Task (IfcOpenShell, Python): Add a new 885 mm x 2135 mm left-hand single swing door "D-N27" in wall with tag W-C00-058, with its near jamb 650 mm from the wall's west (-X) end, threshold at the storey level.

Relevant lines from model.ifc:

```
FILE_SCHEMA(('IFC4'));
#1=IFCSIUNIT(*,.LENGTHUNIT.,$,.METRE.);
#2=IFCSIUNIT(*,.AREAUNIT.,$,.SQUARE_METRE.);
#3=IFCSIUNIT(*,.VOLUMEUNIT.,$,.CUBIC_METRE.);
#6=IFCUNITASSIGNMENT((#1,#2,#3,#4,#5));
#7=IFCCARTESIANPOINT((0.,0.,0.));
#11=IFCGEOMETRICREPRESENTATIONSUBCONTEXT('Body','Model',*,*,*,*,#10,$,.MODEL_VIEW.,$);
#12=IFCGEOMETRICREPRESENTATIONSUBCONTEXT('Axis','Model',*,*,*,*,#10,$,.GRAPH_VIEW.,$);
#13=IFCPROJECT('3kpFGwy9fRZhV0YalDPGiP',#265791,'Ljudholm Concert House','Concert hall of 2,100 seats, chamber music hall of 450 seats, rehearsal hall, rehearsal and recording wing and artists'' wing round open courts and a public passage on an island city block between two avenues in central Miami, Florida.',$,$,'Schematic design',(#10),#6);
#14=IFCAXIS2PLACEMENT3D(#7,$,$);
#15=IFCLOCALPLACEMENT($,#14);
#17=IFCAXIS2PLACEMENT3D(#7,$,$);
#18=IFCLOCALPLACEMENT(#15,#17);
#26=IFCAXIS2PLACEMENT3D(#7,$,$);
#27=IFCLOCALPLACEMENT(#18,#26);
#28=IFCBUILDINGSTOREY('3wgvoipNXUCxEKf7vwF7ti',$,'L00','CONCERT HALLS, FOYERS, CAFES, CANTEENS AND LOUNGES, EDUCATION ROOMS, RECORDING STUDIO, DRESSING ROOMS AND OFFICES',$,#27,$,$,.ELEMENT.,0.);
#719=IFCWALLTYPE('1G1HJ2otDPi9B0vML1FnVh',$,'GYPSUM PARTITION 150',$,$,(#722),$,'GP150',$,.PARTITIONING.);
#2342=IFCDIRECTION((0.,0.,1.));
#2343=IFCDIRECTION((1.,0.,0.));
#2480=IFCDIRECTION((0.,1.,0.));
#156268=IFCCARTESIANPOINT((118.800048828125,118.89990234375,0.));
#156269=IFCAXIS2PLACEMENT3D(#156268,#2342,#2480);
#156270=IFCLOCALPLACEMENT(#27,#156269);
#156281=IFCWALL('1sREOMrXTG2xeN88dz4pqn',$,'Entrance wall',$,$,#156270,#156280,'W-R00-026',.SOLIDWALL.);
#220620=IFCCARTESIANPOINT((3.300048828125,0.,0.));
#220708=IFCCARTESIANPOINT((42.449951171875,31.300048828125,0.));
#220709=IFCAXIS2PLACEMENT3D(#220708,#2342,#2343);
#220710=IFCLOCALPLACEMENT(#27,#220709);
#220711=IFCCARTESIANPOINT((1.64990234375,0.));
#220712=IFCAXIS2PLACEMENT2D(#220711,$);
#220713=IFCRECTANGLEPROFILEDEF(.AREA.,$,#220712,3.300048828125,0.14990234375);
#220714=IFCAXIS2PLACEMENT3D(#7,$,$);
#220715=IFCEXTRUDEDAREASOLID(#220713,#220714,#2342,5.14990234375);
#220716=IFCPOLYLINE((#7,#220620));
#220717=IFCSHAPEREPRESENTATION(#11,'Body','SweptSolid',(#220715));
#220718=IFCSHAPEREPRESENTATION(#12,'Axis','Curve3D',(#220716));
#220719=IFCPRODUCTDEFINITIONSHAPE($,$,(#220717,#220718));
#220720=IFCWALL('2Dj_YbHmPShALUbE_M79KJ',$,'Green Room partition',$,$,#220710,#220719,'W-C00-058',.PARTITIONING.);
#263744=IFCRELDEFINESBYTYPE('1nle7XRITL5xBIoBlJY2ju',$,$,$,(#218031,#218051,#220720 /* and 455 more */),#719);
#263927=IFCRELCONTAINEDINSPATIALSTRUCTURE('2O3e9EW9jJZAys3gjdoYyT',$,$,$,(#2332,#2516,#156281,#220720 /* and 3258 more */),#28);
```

```python
import numpy as np
import ifcopenshell
import ifcopenshell.api.feature
import ifcopenshell.api.geometry
import ifcopenshell.api.root
import ifcopenshell.api.spatial
import ifcopenshell.geom
import ifcopenshell.util.element
import ifcopenshell.util.placement
import ifcopenshell.util.representation
import ifcopenshell.util.shape
import ifcopenshell.util.unit

model = ifcopenshell.open("model.ifc")
unit_scale = ifcopenshell.util.unit.calculate_unit_scale(model)
settings = ifcopenshell.geom.settings()


def volume(element):
    """Net volume in cubic metres, openings subtracted."""
    shape = ifcopenshell.geom.create_shape(settings, element)
    return ifcopenshell.util.shape.get_volume(shape.geometry)


wall = model.by_id(220720)
storey = ifcopenshell.util.element.get_container(wall, ifc_class="IfcBuildingStorey")
context = ifcopenshell.util.representation.get_context(model, "Model", "Body", "MODEL_VIEW")
before = volume(wall)

width, height, from_end, sill = 0.885, 2.135, 0.65, 0.0  # metres

# The wall runs along its own X axis, and the end named is its -X end.
wall_shape = ifcopenshell.geom.create_shape(settings, wall)
x, y, z = ifcopenshell.util.shape.get_vertices(wall_shape.geometry).T
start = x.min() + from_end
face, thickness = float(y.min()), float(y.max() - y.min())
wall_matrix = ifcopenshell.util.placement.get_local_placement(wall.ObjectPlacement)
level = ifcopenshell.util.placement.get_local_placement(storey.ObjectPlacement)[2, 3]


def in_wall(x, y):
    """Placement at x, y metres in the wall's axes, at sill height."""
    matrix = wall_matrix.copy()
    matrix[:, 3] = wall_matrix @ np.array([x / unit_scale, y / unit_scale, 0.0, 1.0])
    matrix[2, 3] = level + sill / unit_scale
    return matrix


# Opening: a box that overshoots both wall faces by 50 mm.
opening = ifcopenshell.api.root.create_entity(model, ifc_class="IfcOpeningElement", predefined_type="OPENING")
box = ifcopenshell.api.geometry.add_wall_representation(
    model, context=context, length=width, height=height, thickness=thickness + 0.1
)
ifcopenshell.api.geometry.assign_representation(model, product=opening, representation=box)
ifcopenshell.api.geometry.edit_object_placement(model, product=opening, matrix=in_wall(start, face - 0.05), is_si=False)
ifcopenshell.api.feature.add_feature(model, feature=opening, element=wall)

door = ifcopenshell.api.root.create_entity(model, ifc_class="IfcDoor", name="D-N27", predefined_type="DOOR")
door.OverallWidth, door.OverallHeight = width / unit_scale, height / unit_scale
door.OperationType = "SINGLE_SWING_LEFT"
body = ifcopenshell.api.geometry.add_door_representation(
    model,
    context=context,
    overall_width=door.OverallWidth,
    overall_height=door.OverallHeight,
    operation_type="SINGLE_SWING_LEFT",
    lining_properties={"LiningDepth": thickness / unit_scale, "ThresholdDepth": thickness / unit_scale},
)
ifcopenshell.api.geometry.assign_representation(model, product=door, representation=body)
ifcopenshell.api.spatial.assign_container(model, products=[door], relating_structure=storey)
ifcopenshell.api.feature.add_filling(model, opening=opening, element=door)

# The lining spans the wall, so the door starts at the wall face.
ifcopenshell.api.geometry.edit_object_placement(model, product=door, matrix=in_wall(start, face), is_si=False)

after = volume(wall)

print(f"wall volume {before:.3f} -> {after:.3f} m3")

model.write("model_rev.ifc")
```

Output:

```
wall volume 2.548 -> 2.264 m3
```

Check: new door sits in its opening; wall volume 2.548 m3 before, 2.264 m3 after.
